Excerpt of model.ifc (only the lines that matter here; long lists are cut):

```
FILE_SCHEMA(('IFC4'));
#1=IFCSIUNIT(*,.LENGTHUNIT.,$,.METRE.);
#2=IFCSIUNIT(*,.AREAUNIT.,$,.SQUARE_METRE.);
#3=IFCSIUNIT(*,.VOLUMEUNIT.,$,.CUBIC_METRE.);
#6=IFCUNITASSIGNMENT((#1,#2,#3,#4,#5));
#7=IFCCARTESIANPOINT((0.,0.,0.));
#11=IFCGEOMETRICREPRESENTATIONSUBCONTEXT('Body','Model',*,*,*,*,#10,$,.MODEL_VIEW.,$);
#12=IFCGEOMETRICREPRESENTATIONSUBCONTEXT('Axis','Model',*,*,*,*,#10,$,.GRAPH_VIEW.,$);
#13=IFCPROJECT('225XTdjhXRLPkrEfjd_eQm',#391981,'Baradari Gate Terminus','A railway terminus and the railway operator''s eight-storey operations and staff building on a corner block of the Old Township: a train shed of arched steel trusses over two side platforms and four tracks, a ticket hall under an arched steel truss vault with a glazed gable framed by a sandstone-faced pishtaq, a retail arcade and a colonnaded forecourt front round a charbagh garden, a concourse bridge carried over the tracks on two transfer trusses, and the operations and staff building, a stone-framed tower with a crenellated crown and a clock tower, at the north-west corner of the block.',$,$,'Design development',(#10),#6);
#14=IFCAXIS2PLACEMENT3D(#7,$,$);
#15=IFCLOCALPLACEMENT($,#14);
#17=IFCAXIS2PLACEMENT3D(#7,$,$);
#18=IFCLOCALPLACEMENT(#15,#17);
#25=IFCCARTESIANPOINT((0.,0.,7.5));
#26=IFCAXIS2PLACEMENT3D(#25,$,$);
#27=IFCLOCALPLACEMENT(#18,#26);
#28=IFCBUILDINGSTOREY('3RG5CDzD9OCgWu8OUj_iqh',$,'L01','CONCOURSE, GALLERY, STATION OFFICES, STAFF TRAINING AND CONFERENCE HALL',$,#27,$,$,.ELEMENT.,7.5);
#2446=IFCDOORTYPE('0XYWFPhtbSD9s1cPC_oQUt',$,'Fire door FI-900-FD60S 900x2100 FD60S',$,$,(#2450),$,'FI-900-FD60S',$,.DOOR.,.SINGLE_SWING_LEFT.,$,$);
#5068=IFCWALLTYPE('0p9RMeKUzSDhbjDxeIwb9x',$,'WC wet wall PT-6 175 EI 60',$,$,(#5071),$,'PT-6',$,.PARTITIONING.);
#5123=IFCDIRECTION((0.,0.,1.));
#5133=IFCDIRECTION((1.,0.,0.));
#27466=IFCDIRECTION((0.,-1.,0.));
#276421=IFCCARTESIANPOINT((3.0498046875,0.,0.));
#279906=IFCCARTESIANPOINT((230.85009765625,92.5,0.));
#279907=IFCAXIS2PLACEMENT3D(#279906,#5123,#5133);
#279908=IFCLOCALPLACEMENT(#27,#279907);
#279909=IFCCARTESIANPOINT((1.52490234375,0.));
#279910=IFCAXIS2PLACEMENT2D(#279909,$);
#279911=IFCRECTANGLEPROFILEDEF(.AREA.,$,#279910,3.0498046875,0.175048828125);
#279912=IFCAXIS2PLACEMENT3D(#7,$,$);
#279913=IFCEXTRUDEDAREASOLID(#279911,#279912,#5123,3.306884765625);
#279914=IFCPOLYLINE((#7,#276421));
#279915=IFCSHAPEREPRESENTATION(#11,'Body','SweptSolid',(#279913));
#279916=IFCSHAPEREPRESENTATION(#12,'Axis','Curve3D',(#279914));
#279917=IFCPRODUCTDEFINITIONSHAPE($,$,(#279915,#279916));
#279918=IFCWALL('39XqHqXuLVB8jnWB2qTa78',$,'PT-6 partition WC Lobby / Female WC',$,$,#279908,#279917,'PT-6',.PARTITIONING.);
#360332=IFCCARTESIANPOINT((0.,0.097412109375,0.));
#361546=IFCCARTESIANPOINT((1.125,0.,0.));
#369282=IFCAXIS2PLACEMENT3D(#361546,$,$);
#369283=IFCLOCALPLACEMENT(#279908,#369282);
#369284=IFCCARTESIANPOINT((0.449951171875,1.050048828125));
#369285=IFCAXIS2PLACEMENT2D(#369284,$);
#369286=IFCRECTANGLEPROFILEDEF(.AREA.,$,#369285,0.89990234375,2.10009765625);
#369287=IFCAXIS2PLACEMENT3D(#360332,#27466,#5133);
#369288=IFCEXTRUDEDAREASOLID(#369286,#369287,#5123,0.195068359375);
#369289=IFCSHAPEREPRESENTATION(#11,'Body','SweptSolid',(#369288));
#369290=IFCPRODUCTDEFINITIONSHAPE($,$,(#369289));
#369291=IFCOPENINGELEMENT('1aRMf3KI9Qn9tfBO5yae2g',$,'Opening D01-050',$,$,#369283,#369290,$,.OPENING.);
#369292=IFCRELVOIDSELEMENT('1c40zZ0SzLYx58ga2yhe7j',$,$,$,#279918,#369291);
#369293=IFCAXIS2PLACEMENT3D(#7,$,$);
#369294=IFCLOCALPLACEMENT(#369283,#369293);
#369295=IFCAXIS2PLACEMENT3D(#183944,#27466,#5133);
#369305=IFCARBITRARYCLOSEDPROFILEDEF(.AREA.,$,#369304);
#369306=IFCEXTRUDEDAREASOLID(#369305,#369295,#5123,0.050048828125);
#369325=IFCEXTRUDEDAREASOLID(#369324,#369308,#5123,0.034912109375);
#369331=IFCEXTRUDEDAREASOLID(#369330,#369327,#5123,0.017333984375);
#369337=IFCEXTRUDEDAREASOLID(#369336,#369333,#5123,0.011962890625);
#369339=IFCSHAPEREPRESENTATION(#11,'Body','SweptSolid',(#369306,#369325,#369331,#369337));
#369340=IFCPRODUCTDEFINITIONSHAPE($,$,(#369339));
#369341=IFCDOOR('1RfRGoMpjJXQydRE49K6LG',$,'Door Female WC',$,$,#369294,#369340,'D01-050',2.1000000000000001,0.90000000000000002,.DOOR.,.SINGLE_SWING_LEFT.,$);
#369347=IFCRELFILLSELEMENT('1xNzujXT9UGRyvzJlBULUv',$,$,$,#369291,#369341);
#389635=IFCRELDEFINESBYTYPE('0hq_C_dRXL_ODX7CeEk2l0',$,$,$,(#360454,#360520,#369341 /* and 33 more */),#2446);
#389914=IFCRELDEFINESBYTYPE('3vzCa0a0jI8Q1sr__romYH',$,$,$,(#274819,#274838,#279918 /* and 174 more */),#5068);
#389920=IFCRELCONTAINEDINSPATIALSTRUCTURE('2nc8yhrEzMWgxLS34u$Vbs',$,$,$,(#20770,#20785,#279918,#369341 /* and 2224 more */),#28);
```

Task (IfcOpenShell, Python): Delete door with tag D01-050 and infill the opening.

```python
import ifcopenshell
import ifcopenshell.api.feature
import ifcopenshell.api.root
import ifcopenshell.geom
import ifcopenshell.util.shape

model = ifcopenshell.open("model.ifc")
settings = ifcopenshell.geom.settings()


def volume(element):
    """Net volume in cubic metres, openings subtracted."""
    shape = ifcopenshell.geom.create_shape(settings, element)
    return ifcopenshell.util.shape.get_volume(shape.geometry)


door = model.by_guid("1RfRGoMpjJXQydRE49K6LG")
opening = door.FillsVoids[0].RelatingOpeningElement
wall = opening.VoidsElements[0].RelatingBuildingElement
before = volume(wall)

ifcopenshell.api.root.remove_product(model, product=door)
ifcopenshell.api.feature.remove_feature(model, feature=opening)

after = volume(wall)

print(f"wall volume {before:.3f} -> {after:.3f} m3")

model.write("model_rev.ifc")
```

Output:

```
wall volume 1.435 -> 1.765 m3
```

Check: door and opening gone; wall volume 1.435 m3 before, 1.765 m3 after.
